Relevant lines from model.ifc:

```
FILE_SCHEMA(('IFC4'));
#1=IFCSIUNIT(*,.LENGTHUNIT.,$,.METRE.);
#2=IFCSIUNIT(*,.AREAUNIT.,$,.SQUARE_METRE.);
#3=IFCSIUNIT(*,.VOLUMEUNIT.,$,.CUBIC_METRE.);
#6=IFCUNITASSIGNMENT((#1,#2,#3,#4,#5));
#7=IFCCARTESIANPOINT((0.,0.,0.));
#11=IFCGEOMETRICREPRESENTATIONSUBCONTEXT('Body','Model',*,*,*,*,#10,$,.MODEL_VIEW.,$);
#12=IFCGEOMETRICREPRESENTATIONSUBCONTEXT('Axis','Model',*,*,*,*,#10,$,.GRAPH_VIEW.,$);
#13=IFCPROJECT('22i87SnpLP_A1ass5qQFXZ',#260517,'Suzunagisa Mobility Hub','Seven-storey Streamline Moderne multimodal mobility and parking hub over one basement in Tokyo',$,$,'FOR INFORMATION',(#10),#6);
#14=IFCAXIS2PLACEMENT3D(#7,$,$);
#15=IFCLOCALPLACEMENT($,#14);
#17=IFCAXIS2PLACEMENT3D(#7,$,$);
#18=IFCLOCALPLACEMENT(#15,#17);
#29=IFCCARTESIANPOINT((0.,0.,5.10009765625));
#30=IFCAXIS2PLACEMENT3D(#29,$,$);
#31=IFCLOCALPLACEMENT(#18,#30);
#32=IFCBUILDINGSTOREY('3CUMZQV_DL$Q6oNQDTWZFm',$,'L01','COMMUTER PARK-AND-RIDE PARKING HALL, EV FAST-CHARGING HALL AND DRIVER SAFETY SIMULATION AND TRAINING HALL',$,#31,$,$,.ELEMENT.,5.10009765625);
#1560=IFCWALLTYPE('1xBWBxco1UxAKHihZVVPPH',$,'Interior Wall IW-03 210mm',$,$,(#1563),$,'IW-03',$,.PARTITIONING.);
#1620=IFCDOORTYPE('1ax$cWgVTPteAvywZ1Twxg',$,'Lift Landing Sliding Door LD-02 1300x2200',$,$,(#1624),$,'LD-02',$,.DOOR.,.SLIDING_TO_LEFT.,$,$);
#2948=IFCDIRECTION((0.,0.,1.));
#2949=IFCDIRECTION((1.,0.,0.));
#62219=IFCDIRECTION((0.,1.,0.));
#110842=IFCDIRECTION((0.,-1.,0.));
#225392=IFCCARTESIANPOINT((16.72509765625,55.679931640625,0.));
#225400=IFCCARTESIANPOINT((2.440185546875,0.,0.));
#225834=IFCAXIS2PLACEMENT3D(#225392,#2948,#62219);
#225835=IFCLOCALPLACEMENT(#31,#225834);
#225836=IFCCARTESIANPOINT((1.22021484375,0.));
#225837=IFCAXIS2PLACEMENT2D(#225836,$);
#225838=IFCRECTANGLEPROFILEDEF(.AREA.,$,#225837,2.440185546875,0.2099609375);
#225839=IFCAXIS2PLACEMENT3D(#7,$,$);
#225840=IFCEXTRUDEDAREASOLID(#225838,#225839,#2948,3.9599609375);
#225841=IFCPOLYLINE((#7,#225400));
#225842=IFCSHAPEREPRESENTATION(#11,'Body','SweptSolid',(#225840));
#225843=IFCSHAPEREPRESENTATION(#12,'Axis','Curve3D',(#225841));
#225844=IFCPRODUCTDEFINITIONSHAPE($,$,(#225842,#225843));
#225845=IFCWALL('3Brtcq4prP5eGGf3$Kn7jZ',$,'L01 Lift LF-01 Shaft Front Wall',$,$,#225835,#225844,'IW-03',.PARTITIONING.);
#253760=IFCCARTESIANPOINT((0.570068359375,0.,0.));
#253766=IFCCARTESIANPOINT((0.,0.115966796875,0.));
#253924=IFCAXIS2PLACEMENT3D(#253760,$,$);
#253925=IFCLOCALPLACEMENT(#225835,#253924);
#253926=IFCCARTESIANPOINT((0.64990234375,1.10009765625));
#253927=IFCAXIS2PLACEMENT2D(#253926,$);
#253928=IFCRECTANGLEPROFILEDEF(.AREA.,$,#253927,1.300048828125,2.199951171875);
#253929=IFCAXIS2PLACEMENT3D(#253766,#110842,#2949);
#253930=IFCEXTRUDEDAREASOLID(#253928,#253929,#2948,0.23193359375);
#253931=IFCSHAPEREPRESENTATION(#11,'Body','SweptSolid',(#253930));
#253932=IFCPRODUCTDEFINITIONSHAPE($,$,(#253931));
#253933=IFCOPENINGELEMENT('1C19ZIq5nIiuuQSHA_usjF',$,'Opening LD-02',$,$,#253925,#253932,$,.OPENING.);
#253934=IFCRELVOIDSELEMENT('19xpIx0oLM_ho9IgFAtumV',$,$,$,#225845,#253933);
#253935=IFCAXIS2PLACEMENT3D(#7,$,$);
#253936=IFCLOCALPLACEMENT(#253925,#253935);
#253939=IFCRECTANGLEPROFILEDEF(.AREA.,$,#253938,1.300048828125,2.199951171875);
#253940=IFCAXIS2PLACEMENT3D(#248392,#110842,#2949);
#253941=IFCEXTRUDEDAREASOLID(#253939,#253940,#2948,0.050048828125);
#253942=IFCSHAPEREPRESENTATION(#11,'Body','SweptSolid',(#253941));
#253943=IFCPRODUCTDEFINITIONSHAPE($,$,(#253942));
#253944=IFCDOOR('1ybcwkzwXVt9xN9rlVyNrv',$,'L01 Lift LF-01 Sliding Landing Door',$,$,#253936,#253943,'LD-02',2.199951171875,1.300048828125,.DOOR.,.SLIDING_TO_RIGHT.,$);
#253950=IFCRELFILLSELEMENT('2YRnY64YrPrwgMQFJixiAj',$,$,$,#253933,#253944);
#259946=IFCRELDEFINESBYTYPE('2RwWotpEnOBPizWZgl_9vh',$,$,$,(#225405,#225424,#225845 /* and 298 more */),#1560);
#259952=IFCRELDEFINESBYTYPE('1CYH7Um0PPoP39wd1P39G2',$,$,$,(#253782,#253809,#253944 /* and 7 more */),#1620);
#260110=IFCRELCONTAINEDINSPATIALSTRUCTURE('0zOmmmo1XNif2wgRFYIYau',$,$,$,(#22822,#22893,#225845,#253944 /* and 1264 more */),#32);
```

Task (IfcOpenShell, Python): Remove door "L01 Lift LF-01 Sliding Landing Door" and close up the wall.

```python
import ifcopenshell
import ifcopenshell.api.feature
import ifcopenshell.api.root
import ifcopenshell.geom
import ifcopenshell.util.shape

model = ifcopenshell.open("model.ifc")
settings = ifcopenshell.geom.settings()


def volume(element):
    """Net volume in cubic metres, openings subtracted."""
    shape = ifcopenshell.geom.create_shape(settings, element)
    return ifcopenshell.util.shape.get_volume(shape.geometry)


door = model.by_id(253944)
opening = door.FillsVoids[0].RelatingOpeningElement
wall = opening.VoidsElements[0].RelatingBuildingElement
before = volume(wall)

ifcopenshell.api.root.remove_product(model, product=door)
ifcopenshell.api.feature.remove_feature(model, feature=opening)

after = volume(wall)

print(f"wall volume {before:.3f} -> {after:.3f} m3")

model.write("model_updated.ifc")
```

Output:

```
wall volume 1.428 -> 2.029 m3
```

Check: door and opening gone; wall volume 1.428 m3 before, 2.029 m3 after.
